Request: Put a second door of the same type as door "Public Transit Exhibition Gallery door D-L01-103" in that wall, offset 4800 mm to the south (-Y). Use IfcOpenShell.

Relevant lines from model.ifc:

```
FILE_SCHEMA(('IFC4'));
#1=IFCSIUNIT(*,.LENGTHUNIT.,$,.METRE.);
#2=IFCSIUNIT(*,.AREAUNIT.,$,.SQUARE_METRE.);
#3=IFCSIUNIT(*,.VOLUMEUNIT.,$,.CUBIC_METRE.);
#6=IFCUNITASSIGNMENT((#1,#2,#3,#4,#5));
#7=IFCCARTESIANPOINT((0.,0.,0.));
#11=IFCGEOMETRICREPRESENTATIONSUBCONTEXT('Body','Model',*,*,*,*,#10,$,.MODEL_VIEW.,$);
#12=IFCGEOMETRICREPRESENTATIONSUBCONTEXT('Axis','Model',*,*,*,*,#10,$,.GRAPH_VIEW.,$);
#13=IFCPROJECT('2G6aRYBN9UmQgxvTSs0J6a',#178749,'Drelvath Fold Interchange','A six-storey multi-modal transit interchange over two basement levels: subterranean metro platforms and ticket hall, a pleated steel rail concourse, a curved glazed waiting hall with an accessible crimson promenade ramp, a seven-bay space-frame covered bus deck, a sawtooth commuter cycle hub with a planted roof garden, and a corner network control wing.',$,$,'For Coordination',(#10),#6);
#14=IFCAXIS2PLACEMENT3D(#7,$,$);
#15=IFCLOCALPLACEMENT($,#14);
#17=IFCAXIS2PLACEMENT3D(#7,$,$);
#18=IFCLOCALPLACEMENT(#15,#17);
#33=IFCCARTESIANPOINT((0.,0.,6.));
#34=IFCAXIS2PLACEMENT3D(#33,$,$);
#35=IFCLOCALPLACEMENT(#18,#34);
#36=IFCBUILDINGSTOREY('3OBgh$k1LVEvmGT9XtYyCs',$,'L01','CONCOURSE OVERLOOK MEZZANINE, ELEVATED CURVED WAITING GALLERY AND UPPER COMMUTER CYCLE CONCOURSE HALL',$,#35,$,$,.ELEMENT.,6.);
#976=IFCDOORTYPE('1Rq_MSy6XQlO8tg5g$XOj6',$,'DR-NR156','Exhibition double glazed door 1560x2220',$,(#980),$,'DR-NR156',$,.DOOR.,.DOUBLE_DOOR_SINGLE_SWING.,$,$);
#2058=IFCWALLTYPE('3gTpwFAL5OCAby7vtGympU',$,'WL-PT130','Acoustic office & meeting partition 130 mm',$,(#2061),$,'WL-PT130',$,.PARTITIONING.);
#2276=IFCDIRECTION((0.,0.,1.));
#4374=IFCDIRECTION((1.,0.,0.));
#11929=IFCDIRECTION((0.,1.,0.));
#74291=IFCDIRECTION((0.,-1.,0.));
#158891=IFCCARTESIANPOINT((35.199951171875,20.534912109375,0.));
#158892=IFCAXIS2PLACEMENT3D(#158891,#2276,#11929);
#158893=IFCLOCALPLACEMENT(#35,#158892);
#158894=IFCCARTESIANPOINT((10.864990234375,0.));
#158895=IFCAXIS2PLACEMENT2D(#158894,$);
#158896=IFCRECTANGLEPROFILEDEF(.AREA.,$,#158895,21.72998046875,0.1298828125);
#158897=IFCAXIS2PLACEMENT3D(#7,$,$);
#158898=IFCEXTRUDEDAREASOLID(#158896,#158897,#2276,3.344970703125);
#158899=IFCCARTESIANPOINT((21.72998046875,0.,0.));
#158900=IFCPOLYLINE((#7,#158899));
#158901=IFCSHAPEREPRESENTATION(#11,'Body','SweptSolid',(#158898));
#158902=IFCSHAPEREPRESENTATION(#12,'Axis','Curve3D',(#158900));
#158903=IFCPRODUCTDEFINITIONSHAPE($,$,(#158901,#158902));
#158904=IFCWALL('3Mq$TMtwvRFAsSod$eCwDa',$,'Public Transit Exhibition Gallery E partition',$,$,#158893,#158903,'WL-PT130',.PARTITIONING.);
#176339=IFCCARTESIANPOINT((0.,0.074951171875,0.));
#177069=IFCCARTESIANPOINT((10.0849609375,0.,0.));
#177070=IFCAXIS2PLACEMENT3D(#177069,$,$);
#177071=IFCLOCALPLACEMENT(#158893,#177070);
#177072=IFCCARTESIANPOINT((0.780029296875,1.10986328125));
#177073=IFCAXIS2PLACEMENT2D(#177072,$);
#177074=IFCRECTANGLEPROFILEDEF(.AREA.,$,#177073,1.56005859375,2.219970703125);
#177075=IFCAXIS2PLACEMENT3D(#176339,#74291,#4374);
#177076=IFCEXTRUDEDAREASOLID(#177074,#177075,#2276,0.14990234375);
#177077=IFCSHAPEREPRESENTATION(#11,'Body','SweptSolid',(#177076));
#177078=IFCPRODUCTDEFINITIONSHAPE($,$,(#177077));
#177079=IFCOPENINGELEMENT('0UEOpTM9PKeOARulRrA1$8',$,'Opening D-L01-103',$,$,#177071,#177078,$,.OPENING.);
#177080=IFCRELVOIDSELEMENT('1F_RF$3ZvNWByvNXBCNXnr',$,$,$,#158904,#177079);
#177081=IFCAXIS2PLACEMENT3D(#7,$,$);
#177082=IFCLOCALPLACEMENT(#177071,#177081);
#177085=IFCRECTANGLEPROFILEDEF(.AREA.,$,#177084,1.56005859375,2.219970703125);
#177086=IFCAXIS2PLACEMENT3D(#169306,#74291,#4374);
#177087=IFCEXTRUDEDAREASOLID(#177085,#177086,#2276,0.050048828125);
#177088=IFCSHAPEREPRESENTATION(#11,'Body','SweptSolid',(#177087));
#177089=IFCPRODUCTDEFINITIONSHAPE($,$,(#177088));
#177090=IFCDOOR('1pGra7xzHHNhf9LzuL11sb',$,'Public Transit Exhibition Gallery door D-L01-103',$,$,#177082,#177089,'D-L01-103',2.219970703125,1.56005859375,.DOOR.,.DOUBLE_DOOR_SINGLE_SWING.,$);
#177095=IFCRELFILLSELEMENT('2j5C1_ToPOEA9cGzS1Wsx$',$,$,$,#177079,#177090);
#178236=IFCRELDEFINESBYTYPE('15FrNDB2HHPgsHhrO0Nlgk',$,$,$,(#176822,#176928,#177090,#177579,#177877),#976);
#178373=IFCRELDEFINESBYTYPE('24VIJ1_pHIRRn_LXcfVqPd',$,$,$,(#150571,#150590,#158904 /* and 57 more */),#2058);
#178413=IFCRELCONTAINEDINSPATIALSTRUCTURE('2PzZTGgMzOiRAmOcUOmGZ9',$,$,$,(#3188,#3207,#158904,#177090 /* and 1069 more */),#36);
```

```python
import ifcopenshell
import ifcopenshell.api.feature
import ifcopenshell.api.geometry
import ifcopenshell.api.root
import ifcopenshell.geom
import ifcopenshell.util.element
import ifcopenshell.util.placement
import ifcopenshell.util.shape
import ifcopenshell.util.unit

model = ifcopenshell.open("model.ifc")
unit_scale = ifcopenshell.util.unit.calculate_unit_scale(model)
settings = ifcopenshell.geom.settings()


def volume(element):
    """Net volume in cubic metres, openings subtracted."""
    shape = ifcopenshell.geom.create_shape(settings, element)
    return ifcopenshell.util.shape.get_volume(shape.geometry)


door = model.by_guid("1pGra7xzHHNhf9LzuL11sb")
opening = door.FillsVoids[0].RelatingOpeningElement
wall = opening.VoidsElements[0].RelatingBuildingElement
before = volume(wall)
shift = ifcopenshell.util.placement.get_local_placement(wall.ObjectPlacement)[:3, 0] * -4.8 / unit_scale

# copy_class copies the void relationship, type, container and properties, but no geometry.
new_opening = ifcopenshell.api.root.copy_class(model, product=opening)
new_opening.Representation = ifcopenshell.util.element.copy_deep(
    model, opening.Representation, exclude=["IfcGeometricRepresentationContext", "IfcRepresentationMap"]
)
new_door = ifcopenshell.api.root.copy_class(model, product=door)
new_door.Representation = ifcopenshell.util.element.copy_deep(
    model, door.Representation, exclude=["IfcGeometricRepresentationContext", "IfcRepresentationMap"]
)
new_door.Tag = None
ifcopenshell.api.feature.add_filling(model, opening=new_opening, element=new_door)

for old, new in ((opening, new_opening), (door, new_door)):
    matrix = ifcopenshell.util.placement.get_local_placement(old.ObjectPlacement)
    matrix[:3, 3] += shift
    ifcopenshell.api.geometry.edit_object_placement(model, product=new, matrix=matrix, is_si=False)

after = volume(wall)

print(f"wall volume {before:.3f} -> {after:.3f} m3")

model.write("model_rev.ifc")
```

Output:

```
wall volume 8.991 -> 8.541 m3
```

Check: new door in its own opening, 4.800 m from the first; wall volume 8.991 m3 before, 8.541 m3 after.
